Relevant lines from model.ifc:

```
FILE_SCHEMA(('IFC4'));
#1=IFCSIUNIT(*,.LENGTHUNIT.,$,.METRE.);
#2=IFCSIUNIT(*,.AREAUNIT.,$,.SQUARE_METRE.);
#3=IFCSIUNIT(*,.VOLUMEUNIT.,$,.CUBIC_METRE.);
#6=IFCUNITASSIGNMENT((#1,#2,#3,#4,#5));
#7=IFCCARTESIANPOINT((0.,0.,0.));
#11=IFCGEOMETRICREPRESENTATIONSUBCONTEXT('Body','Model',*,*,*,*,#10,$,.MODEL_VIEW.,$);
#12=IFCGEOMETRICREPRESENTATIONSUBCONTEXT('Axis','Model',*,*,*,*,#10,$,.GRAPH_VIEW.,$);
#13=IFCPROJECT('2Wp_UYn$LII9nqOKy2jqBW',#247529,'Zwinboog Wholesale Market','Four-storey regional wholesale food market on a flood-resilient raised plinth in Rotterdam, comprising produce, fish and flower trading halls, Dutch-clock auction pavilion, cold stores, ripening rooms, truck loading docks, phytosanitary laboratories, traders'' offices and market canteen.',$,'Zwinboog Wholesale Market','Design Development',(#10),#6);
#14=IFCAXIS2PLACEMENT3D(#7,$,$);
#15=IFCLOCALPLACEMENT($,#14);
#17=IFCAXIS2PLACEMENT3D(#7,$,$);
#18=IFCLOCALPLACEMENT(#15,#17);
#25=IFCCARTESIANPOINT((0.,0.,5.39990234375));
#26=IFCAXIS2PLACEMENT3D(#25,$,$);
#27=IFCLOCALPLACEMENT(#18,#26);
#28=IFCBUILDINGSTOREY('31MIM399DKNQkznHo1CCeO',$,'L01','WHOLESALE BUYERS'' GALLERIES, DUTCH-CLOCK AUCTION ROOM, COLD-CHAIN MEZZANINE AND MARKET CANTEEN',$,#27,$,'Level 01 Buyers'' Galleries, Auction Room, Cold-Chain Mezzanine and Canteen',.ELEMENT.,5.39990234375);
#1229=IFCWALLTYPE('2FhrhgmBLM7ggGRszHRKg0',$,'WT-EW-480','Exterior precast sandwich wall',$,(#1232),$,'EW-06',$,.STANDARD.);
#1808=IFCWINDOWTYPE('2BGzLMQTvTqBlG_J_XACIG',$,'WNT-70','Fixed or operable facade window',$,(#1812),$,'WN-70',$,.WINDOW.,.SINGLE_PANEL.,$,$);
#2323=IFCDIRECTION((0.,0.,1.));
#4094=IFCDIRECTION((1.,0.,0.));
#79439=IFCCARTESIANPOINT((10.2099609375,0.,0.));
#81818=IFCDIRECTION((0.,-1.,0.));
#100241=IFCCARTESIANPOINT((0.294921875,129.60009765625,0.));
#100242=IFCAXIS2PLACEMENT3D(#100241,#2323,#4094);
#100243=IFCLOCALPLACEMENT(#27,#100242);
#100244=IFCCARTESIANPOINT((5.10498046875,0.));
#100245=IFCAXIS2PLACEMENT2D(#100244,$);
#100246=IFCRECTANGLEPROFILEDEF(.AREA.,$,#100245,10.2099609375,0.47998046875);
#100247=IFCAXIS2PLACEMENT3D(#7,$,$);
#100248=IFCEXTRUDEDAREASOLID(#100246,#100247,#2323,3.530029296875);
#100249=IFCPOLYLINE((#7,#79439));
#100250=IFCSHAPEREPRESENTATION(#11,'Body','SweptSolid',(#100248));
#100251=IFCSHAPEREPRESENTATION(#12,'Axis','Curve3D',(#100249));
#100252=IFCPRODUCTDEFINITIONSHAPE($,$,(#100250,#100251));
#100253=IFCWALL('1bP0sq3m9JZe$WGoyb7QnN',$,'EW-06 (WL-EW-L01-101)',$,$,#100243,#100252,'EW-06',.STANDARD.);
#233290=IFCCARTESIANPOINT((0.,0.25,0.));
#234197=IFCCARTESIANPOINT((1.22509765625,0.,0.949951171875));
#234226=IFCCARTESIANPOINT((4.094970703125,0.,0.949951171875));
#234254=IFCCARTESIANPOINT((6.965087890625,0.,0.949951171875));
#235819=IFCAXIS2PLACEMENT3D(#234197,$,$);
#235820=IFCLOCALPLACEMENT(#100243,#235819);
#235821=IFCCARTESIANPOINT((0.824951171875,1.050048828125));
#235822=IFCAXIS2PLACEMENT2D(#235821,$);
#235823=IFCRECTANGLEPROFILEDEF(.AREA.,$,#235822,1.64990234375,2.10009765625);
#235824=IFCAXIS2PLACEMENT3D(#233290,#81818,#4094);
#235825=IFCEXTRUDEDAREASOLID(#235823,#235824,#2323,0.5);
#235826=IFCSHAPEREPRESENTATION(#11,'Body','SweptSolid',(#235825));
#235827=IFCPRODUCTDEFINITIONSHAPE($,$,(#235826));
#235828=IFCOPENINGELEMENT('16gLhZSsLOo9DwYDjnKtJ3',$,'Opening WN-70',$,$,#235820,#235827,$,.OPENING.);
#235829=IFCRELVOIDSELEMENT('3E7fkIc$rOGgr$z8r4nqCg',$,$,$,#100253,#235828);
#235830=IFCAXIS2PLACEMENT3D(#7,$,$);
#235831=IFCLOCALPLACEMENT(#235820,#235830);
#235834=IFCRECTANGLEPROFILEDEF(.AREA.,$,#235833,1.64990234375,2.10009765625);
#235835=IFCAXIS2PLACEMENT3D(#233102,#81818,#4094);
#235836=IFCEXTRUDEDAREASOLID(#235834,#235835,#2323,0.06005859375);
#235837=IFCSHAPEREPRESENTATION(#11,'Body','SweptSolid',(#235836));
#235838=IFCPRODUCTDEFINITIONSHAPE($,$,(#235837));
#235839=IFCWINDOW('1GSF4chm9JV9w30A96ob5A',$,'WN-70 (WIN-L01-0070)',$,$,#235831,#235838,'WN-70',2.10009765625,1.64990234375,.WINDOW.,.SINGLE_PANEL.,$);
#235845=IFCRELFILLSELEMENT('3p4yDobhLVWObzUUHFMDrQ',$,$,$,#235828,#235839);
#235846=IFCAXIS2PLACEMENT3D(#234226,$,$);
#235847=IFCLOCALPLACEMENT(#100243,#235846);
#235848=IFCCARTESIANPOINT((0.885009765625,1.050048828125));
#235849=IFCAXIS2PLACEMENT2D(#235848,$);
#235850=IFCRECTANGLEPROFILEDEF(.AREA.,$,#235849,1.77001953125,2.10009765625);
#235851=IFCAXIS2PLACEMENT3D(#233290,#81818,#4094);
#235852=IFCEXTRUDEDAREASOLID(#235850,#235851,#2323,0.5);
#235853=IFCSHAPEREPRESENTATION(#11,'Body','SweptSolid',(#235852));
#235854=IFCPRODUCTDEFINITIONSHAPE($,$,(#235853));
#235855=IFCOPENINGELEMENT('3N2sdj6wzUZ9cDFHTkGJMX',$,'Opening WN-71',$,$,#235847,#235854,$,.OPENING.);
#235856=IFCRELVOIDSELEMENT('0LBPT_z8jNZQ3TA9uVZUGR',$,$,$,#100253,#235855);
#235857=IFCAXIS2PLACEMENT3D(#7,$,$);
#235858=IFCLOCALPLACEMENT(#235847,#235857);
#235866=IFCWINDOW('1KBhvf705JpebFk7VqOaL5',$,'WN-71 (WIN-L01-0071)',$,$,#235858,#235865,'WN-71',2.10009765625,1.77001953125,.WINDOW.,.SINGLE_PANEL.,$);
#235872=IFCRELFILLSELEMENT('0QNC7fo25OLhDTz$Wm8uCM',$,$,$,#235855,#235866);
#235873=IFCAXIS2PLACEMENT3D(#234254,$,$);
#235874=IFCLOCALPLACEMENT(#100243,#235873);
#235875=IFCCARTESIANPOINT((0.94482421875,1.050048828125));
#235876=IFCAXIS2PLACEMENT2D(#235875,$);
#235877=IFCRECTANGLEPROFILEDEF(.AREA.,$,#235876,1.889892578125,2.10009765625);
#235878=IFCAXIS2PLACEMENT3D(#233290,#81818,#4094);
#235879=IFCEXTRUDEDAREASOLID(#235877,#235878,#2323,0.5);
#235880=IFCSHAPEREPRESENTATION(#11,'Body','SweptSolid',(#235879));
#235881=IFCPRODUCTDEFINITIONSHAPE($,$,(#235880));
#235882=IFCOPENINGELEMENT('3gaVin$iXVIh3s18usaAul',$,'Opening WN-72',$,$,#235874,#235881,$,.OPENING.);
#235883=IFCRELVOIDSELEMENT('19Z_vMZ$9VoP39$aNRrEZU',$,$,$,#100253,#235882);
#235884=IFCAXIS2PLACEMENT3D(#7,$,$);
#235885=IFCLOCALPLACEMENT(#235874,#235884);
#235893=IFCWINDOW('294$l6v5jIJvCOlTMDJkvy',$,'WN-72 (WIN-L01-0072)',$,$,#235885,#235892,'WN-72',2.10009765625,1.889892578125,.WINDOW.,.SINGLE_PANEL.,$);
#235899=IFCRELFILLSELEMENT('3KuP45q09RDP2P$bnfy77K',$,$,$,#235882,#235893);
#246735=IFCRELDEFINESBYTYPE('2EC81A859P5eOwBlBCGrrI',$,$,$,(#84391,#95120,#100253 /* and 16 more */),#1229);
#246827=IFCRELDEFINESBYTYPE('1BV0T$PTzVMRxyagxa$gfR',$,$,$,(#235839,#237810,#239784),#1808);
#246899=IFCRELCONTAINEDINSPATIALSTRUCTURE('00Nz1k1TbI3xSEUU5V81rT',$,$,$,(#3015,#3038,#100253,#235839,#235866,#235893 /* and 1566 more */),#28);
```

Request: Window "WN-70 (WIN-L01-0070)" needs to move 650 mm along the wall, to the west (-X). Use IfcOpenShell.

```python
import ifcopenshell
import ifcopenshell.api.geometry
import ifcopenshell.util.placement
import ifcopenshell.util.unit

model = ifcopenshell.open("model.ifc")
unit_scale = ifcopenshell.util.unit.calculate_unit_scale(model)

window = model.by_guid("1GSF4chm9JV9w30A96ob5A")
opening = window.FillsVoids[0].RelatingOpeningElement
wall = opening.VoidsElements[0].RelatingBuildingElement

wall_matrix = ifcopenshell.util.placement.get_local_placement(wall.ObjectPlacement)
shift = wall_matrix[:3, 0] * -0.65 / unit_scale
before = ifcopenshell.util.placement.get_local_placement(window.ObjectPlacement)[:3, 3].copy()

# The window is placed relative to its opening, so it follows when the opening moves.
matrix = ifcopenshell.util.placement.get_local_placement(opening.ObjectPlacement)
matrix[:3, 3] += shift
ifcopenshell.api.geometry.edit_object_placement(
    model, product=opening, matrix=matrix, is_si=False, should_transform_children=True
)

after = ifcopenshell.util.placement.get_local_placement(window.ObjectPlacement)[:3, 3]
print("window moved by", (after - before).round(3) + 0.0)

model.write("model_updated.ifc")
```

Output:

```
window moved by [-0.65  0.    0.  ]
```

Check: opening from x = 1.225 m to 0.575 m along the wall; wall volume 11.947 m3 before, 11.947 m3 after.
